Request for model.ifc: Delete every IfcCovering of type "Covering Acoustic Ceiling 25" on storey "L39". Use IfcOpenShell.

First a look at what the model holds.

```python
import ifcopenshell
import ifcopenshell.util.element

model = ifcopenshell.open("model.ifc")
print(model.schema)
storey = next(s for s in model.by_type("IfcBuildingStorey") if s.Name == "L39")
coverings = [e for e in ifcopenshell.util.element.get_decomposition(storey) if e.is_a("IfcCovering")]
seen = {}
for e in coverings:
    element_type = ifcopenshell.util.element.get_type(e)
    name = element_type.Name if element_type not in (None, e) else None
    seen[name] = seen.get(name, 0) + 1
for name, count in sorted(seen.items(), key=str):
    print(count, "x", name)
```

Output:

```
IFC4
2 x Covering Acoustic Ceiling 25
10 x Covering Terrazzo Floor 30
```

```python
import ifcopenshell
import ifcopenshell.api.root
import ifcopenshell.util.element

model = ifcopenshell.open("model.ifc")

storey = next(s for s in model.by_type("IfcBuildingStorey") if s.Name == "L39")
coverings = [e for e in ifcopenshell.util.element.get_decomposition(storey) if e.is_a("IfcCovering")]
targets = [e for e in coverings if (t := ifcopenshell.util.element.get_type(e)) not in (None, e) and t.Name == "Covering Acoustic Ceiling 25"]

for e in targets:
    ifcopenshell.api.root.remove_product(model, product=e)
print(len(targets), "removed")

model.write("model_edited.ifc")
```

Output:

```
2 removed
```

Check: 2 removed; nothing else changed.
